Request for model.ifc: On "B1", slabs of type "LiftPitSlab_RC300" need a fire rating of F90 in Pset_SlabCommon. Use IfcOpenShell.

First a look at what the model holds.

```python
import ifcopenshell
import ifcopenshell.util.element

model = ifcopenshell.open("model.ifc")
print(model.schema)
storey = next(s for s in model.by_type("IfcBuildingStorey") if s.Name == "B1")
slabs = [e for e in ifcopenshell.util.element.get_decomposition(storey) if e.is_a("IfcSlab")]
seen = {}
for e in slabs:
    element_type = ifcopenshell.util.element.get_type(e)
    key = (element_type.Name if element_type != e and element_type else None, ifcopenshell.util.element.get_pset(e, "Pset_SlabCommon", "FireRating"))
    seen[key] = seen.get(key, 0) + 1
for (name, value), count in sorted(seen.items(), key=str):
    print(count, "x", name, "|", value)
```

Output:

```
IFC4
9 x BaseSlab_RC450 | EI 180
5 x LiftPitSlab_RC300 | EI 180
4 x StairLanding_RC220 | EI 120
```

```python
import ifcopenshell
import ifcopenshell.api.pset
import ifcopenshell.util.element

model = ifcopenshell.open("model.ifc")

storey = next(s for s in model.by_type("IfcBuildingStorey") if s.Name == "B1")
slabs = [e for e in ifcopenshell.util.element.get_decomposition(storey) if e.is_a("IfcSlab")]

count = 0
for e in slabs:
    element_type = ifcopenshell.util.element.get_type(e)
    if element_type in (None, e) or element_type.Name != "LiftPitSlab_RC300":
        continue
    # add_pset returns the element's existing set when there is one.
    pset = ifcopenshell.api.pset.add_pset(model, product=e, name="Pset_SlabCommon")
    ifcopenshell.api.pset.edit_pset(model, pset=pset, properties={"FireRating": "F90"})
    count += 1

print(count, "slabs updated")

model.write("model_updated.ifc")
```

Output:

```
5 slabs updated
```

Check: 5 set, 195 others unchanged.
